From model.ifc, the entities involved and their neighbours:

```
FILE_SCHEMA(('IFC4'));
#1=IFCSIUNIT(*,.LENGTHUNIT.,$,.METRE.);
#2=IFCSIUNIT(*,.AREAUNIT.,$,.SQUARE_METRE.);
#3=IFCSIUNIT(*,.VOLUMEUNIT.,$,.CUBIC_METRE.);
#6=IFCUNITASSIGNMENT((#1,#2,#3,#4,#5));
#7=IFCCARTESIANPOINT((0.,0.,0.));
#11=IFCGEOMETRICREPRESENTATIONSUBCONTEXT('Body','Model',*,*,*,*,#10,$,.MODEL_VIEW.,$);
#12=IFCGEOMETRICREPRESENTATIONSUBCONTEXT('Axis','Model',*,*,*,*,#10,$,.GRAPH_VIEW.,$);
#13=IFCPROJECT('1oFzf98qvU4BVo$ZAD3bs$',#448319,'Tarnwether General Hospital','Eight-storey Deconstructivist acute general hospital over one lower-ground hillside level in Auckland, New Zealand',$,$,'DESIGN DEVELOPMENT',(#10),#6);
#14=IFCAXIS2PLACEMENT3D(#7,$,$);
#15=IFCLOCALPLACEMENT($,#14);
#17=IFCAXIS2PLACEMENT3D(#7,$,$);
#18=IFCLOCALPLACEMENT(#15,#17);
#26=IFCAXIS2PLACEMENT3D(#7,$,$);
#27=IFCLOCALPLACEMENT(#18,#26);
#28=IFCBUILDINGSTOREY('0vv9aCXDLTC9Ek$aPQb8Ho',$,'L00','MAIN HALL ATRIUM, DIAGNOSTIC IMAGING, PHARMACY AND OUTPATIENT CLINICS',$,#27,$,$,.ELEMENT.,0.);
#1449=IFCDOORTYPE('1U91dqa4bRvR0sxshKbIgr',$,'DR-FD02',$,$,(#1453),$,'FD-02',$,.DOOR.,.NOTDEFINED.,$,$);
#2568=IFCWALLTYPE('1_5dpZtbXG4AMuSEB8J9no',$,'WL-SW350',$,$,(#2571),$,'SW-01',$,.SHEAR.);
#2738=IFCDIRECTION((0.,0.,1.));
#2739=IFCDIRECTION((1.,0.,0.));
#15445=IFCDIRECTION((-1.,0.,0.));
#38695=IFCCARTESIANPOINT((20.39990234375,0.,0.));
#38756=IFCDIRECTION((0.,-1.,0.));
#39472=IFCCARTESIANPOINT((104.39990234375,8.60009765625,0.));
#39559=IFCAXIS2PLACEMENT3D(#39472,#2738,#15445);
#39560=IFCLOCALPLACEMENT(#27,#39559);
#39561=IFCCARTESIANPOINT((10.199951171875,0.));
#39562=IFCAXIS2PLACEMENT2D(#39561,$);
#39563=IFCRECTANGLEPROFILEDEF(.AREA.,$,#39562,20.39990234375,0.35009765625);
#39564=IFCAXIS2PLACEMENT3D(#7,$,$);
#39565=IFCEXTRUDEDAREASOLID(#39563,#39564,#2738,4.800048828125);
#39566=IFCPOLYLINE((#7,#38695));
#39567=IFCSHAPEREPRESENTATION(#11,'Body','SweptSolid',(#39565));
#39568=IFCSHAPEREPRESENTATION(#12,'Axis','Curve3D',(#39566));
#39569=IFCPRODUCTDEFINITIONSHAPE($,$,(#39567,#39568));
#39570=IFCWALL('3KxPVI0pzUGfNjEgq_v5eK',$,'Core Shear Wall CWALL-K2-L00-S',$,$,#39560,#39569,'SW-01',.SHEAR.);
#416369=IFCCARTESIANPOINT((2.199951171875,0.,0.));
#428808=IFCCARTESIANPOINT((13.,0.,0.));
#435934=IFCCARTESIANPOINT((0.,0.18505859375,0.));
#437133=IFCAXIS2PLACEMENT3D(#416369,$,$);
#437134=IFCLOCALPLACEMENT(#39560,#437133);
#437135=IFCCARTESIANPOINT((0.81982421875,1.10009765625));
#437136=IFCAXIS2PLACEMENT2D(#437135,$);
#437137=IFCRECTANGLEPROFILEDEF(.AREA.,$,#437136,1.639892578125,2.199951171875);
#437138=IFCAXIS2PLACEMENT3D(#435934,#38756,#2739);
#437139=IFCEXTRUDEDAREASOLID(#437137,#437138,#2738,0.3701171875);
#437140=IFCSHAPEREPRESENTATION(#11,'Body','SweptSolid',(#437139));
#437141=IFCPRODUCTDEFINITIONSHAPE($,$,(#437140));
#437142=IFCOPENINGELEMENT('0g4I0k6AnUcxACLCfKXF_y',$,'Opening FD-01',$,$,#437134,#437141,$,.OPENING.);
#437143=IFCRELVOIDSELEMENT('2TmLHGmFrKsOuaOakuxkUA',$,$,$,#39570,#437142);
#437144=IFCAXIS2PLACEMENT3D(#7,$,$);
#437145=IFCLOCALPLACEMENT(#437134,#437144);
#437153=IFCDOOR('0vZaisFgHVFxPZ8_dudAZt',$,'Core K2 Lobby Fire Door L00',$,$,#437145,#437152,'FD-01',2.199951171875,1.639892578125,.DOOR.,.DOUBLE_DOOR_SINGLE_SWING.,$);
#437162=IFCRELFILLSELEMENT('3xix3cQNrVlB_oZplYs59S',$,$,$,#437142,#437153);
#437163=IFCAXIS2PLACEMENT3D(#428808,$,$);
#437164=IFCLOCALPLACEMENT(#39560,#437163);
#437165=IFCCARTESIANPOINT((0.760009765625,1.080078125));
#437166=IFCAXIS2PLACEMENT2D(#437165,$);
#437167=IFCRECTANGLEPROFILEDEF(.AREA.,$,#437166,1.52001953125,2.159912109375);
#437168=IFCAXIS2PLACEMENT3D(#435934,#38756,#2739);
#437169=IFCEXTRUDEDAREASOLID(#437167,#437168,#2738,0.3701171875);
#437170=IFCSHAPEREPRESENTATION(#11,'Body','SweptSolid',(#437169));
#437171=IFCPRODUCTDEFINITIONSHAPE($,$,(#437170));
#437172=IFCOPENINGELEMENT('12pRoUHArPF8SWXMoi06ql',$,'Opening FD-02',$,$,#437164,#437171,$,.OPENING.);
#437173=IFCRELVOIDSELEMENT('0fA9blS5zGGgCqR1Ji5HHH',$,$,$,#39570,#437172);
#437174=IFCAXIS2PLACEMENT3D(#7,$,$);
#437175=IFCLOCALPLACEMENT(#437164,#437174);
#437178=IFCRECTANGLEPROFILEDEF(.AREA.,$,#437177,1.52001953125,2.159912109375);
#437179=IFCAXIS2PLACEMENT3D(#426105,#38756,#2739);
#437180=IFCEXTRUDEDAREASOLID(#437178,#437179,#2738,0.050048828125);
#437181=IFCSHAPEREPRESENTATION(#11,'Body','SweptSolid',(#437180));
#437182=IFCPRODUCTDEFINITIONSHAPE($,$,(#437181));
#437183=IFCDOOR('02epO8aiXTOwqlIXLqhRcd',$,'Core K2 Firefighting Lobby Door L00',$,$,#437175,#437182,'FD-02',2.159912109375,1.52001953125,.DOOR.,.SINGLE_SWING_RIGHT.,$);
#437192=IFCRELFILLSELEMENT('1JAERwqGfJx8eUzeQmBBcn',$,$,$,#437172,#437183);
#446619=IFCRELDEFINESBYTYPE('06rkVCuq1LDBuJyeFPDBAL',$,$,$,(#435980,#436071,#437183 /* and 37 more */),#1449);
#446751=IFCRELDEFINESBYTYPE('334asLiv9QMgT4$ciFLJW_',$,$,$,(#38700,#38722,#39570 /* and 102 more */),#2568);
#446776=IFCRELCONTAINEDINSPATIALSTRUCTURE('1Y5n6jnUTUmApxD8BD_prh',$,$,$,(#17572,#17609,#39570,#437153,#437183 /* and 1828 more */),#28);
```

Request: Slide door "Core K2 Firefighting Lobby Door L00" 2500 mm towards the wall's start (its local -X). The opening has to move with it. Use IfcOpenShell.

```python
import ifcopenshell
import ifcopenshell.api.geometry
import ifcopenshell.util.placement
import ifcopenshell.util.unit

model = ifcopenshell.open("model.ifc")
unit_scale = ifcopenshell.util.unit.calculate_unit_scale(model)

door = model.by_guid("02epO8aiXTOwqlIXLqhRcd")
opening = door.FillsVoids[0].RelatingOpeningElement
wall = opening.VoidsElements[0].RelatingBuildingElement

wall_matrix = ifcopenshell.util.placement.get_local_placement(wall.ObjectPlacement)
shift = wall_matrix[:3, 0] * -2.5 / unit_scale
before = ifcopenshell.util.placement.get_local_placement(door.ObjectPlacement)[:3, 3].copy()

# The door is placed relative to its opening, so it follows when the opening moves.
matrix = ifcopenshell.util.placement.get_local_placement(opening.ObjectPlacement)
matrix[:3, 3] += shift
ifcopenshell.api.geometry.edit_object_placement(
    model, product=opening, matrix=matrix, is_si=False, should_transform_children=True
)

after = ifcopenshell.util.placement.get_local_placement(door.ObjectPlacement)[:3, 3]
print("door moved by", (after - before).round(3) + 0.0)

model.write("model_updated.ifc")
```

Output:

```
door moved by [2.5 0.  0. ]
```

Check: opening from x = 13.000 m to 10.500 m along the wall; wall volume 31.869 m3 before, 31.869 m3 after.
